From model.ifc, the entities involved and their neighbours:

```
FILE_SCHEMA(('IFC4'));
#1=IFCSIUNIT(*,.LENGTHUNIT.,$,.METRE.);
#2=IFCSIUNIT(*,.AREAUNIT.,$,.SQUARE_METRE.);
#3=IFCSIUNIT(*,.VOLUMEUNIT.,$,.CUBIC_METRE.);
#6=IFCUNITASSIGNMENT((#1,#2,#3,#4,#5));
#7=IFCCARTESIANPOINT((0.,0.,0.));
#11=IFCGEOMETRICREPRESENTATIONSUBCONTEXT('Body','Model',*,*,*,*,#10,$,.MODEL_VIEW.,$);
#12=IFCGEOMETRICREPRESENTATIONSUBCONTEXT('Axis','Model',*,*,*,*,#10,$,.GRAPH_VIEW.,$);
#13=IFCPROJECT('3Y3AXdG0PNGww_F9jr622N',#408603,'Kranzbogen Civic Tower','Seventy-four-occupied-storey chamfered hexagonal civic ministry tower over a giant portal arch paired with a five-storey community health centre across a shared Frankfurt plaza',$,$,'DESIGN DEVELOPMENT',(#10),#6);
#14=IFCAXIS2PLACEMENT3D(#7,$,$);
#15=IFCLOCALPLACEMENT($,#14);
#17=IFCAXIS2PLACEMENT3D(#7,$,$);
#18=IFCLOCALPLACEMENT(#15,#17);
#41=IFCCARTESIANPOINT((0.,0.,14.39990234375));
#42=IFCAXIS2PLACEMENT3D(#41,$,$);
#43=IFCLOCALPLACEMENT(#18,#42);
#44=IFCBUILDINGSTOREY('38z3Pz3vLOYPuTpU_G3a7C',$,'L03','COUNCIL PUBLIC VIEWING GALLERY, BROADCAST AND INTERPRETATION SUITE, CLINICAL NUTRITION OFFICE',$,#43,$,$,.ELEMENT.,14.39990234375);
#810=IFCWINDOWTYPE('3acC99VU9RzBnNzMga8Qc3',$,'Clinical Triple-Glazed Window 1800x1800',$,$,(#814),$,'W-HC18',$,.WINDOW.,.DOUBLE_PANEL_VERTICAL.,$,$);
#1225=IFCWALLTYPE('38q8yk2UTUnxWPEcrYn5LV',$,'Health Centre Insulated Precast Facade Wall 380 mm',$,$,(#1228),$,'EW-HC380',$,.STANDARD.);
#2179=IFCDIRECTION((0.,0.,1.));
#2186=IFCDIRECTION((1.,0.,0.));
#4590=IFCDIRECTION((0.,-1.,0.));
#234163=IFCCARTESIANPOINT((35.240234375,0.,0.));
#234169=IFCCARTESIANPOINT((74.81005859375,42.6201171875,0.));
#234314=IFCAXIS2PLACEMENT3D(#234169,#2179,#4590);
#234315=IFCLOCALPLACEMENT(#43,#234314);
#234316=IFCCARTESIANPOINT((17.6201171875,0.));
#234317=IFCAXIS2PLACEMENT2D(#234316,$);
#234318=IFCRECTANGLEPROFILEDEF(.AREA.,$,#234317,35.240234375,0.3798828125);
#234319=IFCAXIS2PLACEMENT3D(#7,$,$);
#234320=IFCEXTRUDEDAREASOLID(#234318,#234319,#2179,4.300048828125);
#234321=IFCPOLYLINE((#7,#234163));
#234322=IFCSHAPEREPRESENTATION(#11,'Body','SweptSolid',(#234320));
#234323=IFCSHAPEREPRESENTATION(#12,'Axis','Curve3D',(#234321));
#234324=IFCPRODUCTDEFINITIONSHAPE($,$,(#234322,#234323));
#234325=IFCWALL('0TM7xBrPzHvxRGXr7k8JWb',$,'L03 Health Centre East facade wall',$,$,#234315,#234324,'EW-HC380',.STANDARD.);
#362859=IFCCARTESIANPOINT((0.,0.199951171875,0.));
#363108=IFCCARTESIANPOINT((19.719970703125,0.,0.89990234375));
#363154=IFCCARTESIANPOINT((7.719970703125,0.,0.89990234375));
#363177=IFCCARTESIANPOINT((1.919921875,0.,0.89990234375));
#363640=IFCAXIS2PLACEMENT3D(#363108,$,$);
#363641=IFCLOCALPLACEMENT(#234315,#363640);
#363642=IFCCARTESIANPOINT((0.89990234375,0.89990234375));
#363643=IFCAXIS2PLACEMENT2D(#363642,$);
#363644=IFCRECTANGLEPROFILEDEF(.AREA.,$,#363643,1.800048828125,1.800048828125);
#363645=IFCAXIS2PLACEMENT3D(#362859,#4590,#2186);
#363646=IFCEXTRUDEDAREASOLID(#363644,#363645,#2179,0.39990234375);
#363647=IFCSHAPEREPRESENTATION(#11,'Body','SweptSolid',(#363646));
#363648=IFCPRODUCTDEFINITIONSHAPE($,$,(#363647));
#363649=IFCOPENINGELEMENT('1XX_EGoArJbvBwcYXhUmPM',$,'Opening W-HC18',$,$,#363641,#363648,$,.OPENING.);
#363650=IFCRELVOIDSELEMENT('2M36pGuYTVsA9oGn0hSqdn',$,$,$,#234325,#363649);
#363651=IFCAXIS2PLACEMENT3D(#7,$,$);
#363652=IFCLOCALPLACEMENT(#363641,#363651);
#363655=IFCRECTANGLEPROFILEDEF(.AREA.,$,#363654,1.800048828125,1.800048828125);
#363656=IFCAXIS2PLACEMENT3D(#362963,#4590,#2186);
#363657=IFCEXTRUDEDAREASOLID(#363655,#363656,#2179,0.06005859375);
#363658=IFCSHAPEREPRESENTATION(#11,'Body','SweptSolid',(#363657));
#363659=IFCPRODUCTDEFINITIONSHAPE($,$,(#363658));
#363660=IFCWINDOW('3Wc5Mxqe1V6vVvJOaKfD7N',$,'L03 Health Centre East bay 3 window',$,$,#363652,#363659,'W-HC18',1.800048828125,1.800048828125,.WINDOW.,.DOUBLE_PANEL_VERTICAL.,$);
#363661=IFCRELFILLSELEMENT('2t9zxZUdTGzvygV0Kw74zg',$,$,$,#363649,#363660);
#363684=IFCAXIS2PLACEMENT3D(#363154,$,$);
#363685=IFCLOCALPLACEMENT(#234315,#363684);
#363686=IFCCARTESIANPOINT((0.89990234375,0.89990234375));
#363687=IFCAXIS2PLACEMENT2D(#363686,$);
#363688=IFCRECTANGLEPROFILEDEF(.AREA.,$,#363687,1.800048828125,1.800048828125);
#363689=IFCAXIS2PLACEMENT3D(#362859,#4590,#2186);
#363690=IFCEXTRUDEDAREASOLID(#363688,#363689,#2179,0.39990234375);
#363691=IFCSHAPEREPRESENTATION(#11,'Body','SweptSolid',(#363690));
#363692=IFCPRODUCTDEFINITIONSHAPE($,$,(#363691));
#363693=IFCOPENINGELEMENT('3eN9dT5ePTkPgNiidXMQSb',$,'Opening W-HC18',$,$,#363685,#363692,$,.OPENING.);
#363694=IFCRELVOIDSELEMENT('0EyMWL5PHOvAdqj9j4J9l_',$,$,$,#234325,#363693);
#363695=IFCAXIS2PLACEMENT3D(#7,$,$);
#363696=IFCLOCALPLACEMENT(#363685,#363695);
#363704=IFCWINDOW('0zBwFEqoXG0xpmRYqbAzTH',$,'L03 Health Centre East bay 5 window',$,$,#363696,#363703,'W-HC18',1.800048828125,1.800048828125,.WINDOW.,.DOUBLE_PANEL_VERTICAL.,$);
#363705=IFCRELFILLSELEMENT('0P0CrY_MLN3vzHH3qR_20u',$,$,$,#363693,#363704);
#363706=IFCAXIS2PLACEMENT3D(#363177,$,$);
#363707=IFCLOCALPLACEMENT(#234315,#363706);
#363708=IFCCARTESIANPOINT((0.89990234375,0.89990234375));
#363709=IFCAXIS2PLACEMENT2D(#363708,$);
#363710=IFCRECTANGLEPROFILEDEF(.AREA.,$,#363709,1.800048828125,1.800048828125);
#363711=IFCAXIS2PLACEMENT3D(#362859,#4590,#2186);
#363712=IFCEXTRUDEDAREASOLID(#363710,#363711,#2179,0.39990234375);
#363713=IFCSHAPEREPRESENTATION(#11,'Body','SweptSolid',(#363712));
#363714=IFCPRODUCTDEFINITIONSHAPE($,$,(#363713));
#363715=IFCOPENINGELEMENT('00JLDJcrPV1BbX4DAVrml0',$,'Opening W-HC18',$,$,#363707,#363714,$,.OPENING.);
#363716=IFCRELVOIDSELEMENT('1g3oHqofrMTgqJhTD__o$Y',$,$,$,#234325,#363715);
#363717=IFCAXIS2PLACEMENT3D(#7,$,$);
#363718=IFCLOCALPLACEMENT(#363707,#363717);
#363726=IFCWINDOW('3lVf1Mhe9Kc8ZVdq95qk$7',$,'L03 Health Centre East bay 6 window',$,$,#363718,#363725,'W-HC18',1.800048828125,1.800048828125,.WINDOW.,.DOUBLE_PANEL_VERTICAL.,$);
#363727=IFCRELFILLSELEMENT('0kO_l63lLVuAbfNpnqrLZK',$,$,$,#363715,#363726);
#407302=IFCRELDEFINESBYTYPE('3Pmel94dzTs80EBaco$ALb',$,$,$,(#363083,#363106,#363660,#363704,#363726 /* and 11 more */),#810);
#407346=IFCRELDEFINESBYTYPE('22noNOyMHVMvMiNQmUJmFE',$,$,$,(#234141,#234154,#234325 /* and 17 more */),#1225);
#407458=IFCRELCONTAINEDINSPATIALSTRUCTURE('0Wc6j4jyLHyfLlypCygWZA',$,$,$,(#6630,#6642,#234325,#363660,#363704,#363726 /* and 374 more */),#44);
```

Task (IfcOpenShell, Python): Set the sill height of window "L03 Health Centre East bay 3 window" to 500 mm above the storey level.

```python
import numpy as np
import ifcopenshell
import ifcopenshell.api.geometry
import ifcopenshell.geom
import ifcopenshell.util.element
import ifcopenshell.util.placement
import ifcopenshell.util.shape
import ifcopenshell.util.unit

model = ifcopenshell.open("model.ifc")
unit_scale = ifcopenshell.util.unit.calculate_unit_scale(model)

window = model.by_guid("3Wc5Mxqe1V6vVvJOaKfD7N")
opening = window.FillsVoids[0].RelatingOpeningElement
storey = ifcopenshell.util.element.get_container(window, ifc_class="IfcBuildingStorey")
level = ifcopenshell.util.placement.get_local_placement(storey.ObjectPlacement)[2, 3]

# The opening's origin need not be at the sill, so measure its lowest point.
shape = ifcopenshell.geom.create_shape(ifcopenshell.geom.settings(), opening)
bottom = ifcopenshell.util.shape.get_shape_bottom_elevation(shape, shape.geometry) / unit_scale
dz = level + 0.5 / unit_scale - bottom

shift = np.array([0.0, 0.0, dz])
# The window is placed relative to its opening, so it follows when the opening moves.
matrix = ifcopenshell.util.placement.get_local_placement(opening.ObjectPlacement)
matrix[:3, 3] += shift
ifcopenshell.api.geometry.edit_object_placement(
    model, product=opening, matrix=matrix, is_si=False, should_transform_children=True
)

print(f"moved by {dz * unit_scale:+.3f} m")

model.write("model_v2.ifc")
```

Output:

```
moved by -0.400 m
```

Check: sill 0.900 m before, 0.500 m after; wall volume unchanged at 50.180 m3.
